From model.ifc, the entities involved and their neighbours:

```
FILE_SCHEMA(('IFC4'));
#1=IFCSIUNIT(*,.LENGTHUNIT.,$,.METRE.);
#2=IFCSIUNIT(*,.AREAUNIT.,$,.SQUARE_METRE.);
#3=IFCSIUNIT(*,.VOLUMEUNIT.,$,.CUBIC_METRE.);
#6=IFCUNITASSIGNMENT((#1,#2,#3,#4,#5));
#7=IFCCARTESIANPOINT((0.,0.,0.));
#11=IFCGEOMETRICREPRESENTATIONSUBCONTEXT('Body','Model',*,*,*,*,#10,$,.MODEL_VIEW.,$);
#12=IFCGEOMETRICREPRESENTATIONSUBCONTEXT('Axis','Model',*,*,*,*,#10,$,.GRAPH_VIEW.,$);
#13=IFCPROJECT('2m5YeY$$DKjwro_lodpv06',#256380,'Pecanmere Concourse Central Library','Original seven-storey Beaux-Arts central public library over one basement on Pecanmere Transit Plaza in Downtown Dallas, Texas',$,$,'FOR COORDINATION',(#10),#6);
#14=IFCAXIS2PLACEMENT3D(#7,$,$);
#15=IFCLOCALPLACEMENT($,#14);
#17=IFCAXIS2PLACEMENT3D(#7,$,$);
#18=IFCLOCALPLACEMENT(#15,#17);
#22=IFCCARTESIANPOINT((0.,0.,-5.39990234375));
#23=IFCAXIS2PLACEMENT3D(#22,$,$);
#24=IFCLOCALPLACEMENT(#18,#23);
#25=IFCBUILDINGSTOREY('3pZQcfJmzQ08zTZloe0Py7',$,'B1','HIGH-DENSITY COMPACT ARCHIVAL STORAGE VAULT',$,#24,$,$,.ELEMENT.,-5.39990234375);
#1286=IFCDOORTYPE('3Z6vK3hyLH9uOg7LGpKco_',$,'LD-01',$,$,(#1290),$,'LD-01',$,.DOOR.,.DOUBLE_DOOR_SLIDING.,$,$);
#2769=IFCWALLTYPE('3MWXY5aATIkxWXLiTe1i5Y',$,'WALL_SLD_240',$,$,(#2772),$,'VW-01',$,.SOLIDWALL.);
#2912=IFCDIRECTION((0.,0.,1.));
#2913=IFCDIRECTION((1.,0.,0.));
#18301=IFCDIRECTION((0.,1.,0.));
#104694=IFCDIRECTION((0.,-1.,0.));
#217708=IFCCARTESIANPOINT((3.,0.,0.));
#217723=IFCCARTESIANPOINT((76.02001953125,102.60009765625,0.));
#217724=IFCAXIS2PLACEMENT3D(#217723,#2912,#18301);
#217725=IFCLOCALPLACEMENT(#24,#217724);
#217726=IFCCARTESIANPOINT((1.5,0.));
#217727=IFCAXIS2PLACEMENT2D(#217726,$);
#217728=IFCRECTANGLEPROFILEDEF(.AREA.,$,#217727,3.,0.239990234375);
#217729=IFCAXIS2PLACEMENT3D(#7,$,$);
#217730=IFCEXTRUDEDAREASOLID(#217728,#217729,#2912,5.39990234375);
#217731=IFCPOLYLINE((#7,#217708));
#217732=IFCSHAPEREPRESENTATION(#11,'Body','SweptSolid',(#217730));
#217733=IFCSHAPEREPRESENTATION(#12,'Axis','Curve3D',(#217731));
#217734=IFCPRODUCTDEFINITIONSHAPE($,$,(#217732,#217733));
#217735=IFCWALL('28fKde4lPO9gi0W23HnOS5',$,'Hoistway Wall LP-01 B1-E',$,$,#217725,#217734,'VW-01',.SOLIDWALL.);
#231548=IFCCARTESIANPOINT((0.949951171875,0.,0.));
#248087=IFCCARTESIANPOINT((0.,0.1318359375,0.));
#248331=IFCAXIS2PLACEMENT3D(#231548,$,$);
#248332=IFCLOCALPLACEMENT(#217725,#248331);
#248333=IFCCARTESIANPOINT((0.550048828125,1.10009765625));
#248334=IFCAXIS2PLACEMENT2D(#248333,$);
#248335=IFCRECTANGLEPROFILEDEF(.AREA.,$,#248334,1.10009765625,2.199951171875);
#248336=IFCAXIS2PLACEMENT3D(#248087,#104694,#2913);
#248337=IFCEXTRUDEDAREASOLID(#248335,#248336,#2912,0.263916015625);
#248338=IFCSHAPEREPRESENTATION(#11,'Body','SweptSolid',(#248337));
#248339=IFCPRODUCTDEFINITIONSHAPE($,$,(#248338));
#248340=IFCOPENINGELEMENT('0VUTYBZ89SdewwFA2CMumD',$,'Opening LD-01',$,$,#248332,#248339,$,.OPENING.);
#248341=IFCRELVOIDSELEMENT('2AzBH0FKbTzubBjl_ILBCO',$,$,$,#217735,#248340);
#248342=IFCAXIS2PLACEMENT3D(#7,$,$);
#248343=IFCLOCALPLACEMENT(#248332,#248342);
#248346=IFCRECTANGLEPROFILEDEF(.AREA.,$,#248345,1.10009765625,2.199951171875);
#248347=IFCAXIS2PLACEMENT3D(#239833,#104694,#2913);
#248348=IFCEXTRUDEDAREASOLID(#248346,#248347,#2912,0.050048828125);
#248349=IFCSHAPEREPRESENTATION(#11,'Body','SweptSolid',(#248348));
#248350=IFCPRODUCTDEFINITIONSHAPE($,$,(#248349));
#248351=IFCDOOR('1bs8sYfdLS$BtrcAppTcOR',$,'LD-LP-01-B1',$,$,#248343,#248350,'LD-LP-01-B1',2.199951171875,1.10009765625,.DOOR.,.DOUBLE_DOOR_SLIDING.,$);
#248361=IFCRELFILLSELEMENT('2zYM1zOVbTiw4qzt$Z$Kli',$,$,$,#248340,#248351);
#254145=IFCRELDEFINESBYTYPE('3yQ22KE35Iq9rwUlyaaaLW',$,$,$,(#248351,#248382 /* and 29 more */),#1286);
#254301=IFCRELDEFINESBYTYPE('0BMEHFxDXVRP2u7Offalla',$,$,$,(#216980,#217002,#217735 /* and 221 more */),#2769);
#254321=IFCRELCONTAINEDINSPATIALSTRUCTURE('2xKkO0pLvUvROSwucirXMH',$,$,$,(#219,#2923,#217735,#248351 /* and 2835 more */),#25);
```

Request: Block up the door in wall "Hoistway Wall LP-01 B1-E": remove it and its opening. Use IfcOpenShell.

```python
import ifcopenshell
import ifcopenshell.api.feature
import ifcopenshell.api.root
import ifcopenshell.geom
import ifcopenshell.util.shape

model = ifcopenshell.open("model.ifc")
settings = ifcopenshell.geom.settings()


def volume(element):
    """Net volume in cubic metres, openings subtracted."""
    shape = ifcopenshell.geom.create_shape(settings, element)
    return ifcopenshell.util.shape.get_volume(shape.geometry)


door = model.by_guid("1bs8sYfdLS$BtrcAppTcOR")
opening = door.FillsVoids[0].RelatingOpeningElement
wall = opening.VoidsElements[0].RelatingBuildingElement
before = volume(wall)

ifcopenshell.api.root.remove_product(model, product=door)
ifcopenshell.api.feature.remove_feature(model, feature=opening)

after = volume(wall)

print(f"wall volume {before:.3f} -> {after:.3f} m3")

model.write("model_rev.ifc")
```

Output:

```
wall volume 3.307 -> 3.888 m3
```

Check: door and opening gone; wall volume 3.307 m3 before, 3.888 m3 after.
